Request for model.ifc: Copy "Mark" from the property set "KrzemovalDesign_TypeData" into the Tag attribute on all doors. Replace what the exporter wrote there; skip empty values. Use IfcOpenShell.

First a look at what the model holds.

```python
import ifcopenshell
import ifcopenshell.util.element

model = ifcopenshell.open("model.ifc")
print(model.schema)
doors = model.by_type("IfcDoor")
print(len(doors), "doors")
for e in doors[:8]:
    source = ifcopenshell.util.element.get_pset(e, "KrzemovalDesign_TypeData", "Mark")
    target = e.Tag
    print(e.id(), repr(source), repr(target), sep=" | ")
```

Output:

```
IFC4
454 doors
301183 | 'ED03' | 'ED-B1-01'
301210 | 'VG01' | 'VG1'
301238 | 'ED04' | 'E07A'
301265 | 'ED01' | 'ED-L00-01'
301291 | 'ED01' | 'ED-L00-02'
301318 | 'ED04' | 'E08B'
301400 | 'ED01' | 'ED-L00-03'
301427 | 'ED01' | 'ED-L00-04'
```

```python
import ifcopenshell
import ifcopenshell.util.element

model = ifcopenshell.open("model.ifc")

count = 0
for e in model.by_type("IfcDoor"):
    value = ifcopenshell.util.element.get_pset(e, "KrzemovalDesign_TypeData", "Mark")
    current = e.Tag
    if not value or not value.strip() or current == value:
        continue
    e.Tag = value
    count += 1

print(count, "doors updated")

model.write("model_rev.ifc")
```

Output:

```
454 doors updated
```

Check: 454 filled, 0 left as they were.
